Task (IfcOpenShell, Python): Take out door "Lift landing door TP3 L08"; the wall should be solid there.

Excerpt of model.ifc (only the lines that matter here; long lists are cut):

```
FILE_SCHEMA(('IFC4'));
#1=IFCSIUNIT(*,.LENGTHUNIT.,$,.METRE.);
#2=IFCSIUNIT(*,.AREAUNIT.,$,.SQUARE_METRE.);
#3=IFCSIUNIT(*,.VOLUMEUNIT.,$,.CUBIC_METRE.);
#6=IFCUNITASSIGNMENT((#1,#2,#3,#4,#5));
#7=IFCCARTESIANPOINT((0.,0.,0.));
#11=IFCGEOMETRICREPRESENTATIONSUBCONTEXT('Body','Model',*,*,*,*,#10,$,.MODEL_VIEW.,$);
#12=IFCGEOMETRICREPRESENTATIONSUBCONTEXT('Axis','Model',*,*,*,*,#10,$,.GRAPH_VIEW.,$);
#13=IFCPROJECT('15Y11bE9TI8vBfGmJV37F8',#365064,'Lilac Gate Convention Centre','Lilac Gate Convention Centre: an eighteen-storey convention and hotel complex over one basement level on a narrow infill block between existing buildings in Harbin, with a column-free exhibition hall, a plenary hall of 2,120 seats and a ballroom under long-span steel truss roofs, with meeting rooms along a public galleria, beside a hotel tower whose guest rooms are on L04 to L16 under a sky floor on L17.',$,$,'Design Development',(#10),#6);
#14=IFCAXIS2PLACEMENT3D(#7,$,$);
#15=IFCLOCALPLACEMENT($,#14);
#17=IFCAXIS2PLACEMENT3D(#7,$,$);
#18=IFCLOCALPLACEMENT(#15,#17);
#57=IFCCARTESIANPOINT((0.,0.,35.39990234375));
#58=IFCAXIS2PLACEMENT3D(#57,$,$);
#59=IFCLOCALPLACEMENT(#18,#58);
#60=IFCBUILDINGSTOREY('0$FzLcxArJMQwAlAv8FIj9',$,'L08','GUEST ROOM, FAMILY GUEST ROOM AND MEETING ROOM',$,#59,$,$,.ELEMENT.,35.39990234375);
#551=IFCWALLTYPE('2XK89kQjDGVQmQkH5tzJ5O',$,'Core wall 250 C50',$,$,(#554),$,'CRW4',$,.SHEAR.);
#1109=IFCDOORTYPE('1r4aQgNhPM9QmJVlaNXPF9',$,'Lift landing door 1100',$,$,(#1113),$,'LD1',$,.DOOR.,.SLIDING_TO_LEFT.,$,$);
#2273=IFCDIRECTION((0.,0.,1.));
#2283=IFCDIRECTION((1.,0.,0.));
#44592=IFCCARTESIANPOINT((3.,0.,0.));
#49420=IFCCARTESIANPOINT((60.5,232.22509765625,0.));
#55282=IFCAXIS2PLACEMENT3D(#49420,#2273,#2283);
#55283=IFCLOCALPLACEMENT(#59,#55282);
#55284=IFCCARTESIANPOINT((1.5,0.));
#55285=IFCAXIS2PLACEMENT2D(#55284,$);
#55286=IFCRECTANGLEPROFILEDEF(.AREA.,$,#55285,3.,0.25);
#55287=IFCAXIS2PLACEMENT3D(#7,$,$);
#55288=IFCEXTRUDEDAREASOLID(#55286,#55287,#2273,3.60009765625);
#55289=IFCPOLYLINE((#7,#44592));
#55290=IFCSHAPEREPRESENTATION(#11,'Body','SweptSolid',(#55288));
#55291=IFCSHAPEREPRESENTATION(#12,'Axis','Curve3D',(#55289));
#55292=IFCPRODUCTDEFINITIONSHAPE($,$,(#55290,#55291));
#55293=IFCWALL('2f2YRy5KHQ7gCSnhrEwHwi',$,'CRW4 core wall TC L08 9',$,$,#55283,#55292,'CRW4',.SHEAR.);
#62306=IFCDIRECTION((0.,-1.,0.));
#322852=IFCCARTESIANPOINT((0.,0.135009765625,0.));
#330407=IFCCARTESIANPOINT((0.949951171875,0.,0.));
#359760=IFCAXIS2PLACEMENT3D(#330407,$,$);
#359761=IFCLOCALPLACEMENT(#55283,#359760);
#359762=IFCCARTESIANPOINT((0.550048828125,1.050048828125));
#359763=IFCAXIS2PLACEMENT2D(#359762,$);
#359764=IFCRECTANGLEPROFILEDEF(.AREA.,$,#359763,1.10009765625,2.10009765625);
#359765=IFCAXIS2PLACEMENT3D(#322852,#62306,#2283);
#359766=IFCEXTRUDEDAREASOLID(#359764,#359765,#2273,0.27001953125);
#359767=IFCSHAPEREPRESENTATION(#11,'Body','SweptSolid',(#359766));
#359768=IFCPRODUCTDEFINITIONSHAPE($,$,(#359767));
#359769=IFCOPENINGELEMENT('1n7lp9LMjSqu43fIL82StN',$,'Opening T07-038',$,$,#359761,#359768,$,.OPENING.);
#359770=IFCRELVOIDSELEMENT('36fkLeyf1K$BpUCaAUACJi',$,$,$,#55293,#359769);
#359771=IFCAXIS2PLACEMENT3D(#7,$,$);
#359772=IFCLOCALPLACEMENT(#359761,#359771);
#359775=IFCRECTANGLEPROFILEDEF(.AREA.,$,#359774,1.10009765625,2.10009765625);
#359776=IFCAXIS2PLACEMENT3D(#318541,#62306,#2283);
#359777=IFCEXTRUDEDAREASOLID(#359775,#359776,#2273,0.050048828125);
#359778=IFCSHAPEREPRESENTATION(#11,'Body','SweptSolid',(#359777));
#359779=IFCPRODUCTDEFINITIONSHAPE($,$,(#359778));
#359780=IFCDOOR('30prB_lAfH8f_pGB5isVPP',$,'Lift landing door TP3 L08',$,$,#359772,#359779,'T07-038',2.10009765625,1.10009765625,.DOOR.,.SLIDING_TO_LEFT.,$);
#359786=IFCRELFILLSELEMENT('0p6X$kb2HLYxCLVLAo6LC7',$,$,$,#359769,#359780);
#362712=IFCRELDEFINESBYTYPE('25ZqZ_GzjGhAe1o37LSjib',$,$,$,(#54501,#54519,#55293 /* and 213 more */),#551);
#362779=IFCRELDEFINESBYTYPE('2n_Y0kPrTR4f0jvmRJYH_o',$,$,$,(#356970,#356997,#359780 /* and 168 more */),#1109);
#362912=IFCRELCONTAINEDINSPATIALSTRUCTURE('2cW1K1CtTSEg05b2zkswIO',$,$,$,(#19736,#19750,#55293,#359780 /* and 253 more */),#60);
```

```python
import ifcopenshell
import ifcopenshell.api.feature
import ifcopenshell.api.root
import ifcopenshell.geom
import ifcopenshell.util.shape

model = ifcopenshell.open("model.ifc")
settings = ifcopenshell.geom.settings()


def volume(element):
    """Net volume in cubic metres, openings subtracted."""
    shape = ifcopenshell.geom.create_shape(settings, element)
    return ifcopenshell.util.shape.get_volume(shape.geometry)


door = model.by_id(359780)
opening = door.FillsVoids[0].RelatingOpeningElement
wall = opening.VoidsElements[0].RelatingBuildingElement
before = volume(wall)

ifcopenshell.api.root.remove_product(model, product=door)
ifcopenshell.api.feature.remove_feature(model, feature=opening)

after = volume(wall)

print(f"wall volume {before:.3f} -> {after:.3f} m3")

model.write("model_updated.ifc")
```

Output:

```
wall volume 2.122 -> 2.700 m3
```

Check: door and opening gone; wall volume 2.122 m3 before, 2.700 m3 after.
